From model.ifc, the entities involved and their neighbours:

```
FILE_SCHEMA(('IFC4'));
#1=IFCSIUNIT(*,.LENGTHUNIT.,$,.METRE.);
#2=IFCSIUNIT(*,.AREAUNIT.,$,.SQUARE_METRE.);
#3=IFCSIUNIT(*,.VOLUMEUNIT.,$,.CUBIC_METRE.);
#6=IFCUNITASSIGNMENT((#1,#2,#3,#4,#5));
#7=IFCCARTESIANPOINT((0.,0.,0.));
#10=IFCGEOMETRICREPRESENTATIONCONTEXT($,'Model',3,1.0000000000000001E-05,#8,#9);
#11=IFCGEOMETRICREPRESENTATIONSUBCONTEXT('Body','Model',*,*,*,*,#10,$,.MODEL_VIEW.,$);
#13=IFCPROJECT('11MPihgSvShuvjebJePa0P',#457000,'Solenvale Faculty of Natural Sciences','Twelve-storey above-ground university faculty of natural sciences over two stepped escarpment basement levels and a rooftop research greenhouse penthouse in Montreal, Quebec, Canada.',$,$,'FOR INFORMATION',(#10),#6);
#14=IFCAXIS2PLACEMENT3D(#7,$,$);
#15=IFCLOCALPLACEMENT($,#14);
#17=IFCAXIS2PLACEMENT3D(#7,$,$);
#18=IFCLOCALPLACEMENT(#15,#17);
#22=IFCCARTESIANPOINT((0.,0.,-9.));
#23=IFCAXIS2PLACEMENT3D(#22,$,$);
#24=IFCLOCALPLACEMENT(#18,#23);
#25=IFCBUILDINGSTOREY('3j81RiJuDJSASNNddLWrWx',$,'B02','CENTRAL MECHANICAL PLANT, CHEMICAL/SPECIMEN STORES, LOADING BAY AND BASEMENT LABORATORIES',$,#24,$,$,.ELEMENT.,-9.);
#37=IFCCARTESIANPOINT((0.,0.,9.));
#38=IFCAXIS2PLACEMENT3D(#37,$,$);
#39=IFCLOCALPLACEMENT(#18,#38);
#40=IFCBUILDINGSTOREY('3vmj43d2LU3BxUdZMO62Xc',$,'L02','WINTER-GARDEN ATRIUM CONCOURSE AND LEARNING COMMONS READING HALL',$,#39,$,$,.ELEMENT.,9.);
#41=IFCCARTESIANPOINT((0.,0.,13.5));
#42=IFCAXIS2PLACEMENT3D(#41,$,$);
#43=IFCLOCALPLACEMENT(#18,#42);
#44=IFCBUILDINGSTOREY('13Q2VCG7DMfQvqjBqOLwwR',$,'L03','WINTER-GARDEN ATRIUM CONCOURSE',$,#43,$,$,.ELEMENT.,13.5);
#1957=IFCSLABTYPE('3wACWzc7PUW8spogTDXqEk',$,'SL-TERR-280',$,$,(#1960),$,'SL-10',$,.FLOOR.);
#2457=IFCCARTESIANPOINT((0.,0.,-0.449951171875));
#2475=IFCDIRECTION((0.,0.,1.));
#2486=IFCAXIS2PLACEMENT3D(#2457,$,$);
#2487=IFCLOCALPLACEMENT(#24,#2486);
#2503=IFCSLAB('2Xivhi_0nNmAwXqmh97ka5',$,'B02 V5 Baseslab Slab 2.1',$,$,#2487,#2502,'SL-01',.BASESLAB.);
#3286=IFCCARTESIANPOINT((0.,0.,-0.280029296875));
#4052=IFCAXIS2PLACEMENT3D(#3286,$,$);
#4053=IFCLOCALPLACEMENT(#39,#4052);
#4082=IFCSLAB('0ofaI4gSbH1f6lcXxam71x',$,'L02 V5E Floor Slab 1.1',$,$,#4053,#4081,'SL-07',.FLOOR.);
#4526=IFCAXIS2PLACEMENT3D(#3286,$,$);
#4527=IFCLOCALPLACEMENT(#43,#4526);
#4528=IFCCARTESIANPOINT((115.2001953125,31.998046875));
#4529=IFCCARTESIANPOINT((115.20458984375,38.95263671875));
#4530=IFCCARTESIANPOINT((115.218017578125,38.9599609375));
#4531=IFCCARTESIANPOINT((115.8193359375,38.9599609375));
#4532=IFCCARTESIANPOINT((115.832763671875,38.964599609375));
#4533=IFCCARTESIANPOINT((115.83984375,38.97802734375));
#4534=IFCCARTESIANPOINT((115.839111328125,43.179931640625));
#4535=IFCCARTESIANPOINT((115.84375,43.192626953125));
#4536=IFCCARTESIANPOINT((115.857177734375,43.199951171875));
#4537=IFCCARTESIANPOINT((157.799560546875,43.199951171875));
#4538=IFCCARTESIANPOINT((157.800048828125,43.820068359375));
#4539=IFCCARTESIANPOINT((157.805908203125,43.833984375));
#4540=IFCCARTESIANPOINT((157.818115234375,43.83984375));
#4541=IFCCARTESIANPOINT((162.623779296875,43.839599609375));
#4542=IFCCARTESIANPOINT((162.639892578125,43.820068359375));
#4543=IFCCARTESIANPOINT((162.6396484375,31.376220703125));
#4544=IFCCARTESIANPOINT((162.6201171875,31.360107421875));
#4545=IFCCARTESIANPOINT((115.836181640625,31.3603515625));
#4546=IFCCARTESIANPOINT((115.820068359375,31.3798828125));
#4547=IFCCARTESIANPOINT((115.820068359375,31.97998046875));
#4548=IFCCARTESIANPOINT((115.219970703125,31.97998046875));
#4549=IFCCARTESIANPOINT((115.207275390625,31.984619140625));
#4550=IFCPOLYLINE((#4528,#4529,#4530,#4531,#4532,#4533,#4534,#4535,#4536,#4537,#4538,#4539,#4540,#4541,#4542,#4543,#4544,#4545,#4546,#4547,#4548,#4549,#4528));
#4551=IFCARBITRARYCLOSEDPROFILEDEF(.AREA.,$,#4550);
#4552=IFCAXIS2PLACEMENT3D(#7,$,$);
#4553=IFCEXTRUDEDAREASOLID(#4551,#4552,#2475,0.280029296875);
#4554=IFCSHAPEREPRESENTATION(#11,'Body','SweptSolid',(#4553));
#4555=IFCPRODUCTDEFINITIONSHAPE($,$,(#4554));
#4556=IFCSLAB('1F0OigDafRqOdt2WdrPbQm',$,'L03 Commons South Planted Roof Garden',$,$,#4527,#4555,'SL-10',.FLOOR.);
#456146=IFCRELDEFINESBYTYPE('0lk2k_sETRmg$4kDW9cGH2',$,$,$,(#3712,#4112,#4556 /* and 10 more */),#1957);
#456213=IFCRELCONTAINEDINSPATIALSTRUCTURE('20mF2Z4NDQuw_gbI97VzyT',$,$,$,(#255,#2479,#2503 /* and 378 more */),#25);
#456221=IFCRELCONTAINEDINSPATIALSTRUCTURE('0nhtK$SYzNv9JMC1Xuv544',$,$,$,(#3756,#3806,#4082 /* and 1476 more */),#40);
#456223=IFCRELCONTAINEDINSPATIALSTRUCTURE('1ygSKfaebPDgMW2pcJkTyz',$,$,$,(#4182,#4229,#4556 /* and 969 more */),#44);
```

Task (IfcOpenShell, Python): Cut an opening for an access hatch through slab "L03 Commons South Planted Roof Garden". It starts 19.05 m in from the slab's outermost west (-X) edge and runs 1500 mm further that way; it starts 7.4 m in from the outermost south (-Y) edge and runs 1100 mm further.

```python
import numpy as np
import ifcopenshell
import ifcopenshell.api.feature
import ifcopenshell.api.geometry
import ifcopenshell.api.root
import ifcopenshell.geom
import ifcopenshell.util.placement
import ifcopenshell.util.representation
import ifcopenshell.util.shape
import ifcopenshell.util.unit

model = ifcopenshell.open("model.ifc")
unit_scale = ifcopenshell.util.unit.calculate_unit_scale(model)
settings = ifcopenshell.geom.settings()


def volume(element):
    """Net volume in cubic metres, openings subtracted."""
    shape = ifcopenshell.geom.create_shape(settings, element)
    return ifcopenshell.util.shape.get_volume(shape.geometry)


slab = model.by_guid("1F0OigDafRqOdt2WdrPbQm")
before = volume(slab)

# Extent in the slab's own axes, in metres. The edges named are its -X and -Y sides.
slab_shape = ifcopenshell.geom.create_shape(settings, slab)
vertices = ifcopenshell.util.shape.get_vertices(slab_shape.geometry)
x_min, y_min, bottom = vertices.min(axis=0)
top = vertices[:, 2].max()

opening = ifcopenshell.api.root.create_entity(model, ifc_class="IfcOpeningElement", name="Access hatch opening", predefined_type="OPENING")
context = ifcopenshell.util.representation.get_context(model, "Model", "Body", "MODEL_VIEW")
width, depth = 1.5, 1.1
outline = [(0.0, 0.0), (width, 0.0), (width, depth), (0.0, depth), (0.0, 0.0)]
# Overshoot both faces by 50 mm so the cut is clean.
shape = ifcopenshell.api.geometry.add_slab_representation(
    model, context=context, depth=top - bottom + 0.1, polyline=outline
)
ifcopenshell.api.geometry.assign_representation(model, product=opening, representation=shape)

matrix = ifcopenshell.util.placement.get_local_placement(slab.ObjectPlacement)
matrix[:, 3] = matrix @ np.append(np.array([x_min + 19.05, y_min + 7.4, bottom - 0.05]) / unit_scale, 1.0)
ifcopenshell.api.geometry.edit_object_placement(model, product=opening, matrix=matrix, is_si=False)
ifcopenshell.api.feature.add_feature(model, feature=opening, element=slab)

after = volume(slab)

print(f"slab volume {before:.3f} -> {after:.3f} m3")

model.write("model-out.ifc")
```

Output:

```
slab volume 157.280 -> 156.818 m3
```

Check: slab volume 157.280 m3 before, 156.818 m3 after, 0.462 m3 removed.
